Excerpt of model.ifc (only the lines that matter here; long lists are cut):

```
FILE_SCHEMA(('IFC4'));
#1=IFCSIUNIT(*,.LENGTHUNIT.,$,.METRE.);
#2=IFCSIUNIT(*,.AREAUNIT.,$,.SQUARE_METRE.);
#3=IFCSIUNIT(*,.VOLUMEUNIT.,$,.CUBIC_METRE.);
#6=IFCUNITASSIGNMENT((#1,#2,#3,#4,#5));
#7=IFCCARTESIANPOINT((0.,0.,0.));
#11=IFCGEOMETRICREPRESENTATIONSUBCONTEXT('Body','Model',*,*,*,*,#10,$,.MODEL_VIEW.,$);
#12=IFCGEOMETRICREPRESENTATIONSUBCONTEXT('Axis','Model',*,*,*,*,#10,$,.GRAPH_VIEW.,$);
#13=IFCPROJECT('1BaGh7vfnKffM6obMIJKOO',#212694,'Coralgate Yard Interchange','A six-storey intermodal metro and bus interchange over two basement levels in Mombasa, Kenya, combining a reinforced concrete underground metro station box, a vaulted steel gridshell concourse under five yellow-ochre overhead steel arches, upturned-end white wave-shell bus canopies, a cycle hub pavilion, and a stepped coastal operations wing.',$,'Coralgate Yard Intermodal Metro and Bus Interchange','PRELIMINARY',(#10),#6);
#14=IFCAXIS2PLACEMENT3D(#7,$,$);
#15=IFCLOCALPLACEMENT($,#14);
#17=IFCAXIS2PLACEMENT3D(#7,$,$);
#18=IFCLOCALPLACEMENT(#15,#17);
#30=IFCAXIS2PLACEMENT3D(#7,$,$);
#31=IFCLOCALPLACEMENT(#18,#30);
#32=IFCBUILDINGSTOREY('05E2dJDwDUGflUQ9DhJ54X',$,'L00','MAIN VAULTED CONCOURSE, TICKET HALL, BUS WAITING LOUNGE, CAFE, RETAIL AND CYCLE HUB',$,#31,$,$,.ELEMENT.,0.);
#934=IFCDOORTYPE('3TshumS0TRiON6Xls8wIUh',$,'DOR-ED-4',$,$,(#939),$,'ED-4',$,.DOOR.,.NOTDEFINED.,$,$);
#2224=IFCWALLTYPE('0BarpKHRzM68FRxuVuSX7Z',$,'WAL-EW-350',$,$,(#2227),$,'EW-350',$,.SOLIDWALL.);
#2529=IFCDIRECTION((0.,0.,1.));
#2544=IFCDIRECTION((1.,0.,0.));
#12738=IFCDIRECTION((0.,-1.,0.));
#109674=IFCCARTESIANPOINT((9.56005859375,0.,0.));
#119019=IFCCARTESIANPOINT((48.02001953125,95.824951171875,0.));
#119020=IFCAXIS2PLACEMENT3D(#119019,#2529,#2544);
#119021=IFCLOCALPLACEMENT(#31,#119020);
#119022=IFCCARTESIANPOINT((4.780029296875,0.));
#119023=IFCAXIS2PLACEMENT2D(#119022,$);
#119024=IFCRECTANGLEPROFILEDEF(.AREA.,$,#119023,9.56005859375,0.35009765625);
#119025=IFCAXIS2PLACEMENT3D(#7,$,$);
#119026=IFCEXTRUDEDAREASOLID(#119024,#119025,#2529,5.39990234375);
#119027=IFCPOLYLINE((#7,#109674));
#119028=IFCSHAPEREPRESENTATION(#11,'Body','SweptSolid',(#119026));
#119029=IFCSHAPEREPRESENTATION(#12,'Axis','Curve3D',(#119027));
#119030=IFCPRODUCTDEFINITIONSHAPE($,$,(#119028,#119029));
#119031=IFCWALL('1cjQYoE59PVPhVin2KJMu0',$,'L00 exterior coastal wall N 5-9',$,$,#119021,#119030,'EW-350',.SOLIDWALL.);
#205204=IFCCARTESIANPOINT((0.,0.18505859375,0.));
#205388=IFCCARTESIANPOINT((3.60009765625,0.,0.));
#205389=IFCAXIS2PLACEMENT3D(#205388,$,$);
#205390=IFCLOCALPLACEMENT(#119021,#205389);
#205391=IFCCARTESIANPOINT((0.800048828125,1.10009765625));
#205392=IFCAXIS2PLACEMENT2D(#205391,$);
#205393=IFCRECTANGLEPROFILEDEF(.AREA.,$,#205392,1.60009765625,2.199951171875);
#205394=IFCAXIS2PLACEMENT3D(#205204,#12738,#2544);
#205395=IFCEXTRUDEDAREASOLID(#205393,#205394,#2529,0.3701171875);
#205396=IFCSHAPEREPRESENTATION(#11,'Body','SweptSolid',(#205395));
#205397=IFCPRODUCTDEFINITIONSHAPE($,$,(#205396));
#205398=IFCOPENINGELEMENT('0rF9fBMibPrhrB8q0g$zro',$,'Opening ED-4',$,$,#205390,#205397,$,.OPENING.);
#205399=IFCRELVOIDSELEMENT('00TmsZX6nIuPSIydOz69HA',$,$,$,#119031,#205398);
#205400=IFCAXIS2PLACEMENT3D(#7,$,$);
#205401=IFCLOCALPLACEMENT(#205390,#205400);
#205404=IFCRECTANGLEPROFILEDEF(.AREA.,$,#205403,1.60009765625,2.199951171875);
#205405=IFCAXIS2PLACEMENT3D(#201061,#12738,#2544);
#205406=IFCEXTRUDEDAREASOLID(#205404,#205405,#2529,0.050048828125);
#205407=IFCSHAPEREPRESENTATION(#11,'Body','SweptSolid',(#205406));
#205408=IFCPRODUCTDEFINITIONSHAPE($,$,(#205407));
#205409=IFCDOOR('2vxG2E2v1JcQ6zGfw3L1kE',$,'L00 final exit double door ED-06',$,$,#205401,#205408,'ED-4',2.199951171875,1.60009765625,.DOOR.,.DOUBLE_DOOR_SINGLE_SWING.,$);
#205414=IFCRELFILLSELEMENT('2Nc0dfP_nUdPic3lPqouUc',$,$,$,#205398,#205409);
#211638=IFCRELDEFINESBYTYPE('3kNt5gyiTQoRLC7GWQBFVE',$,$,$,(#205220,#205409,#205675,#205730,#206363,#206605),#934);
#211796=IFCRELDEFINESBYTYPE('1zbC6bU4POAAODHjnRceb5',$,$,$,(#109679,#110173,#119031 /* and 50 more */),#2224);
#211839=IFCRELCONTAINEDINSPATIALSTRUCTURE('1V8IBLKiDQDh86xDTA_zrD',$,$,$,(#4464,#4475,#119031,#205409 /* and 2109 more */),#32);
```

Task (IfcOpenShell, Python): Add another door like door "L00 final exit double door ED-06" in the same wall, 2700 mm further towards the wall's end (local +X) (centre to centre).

```python
import ifcopenshell
import ifcopenshell.api.feature
import ifcopenshell.api.geometry
import ifcopenshell.api.root
import ifcopenshell.geom
import ifcopenshell.util.element
import ifcopenshell.util.placement
import ifcopenshell.util.shape

model = ifcopenshell.open("model.ifc")
settings = ifcopenshell.geom.settings()


def volume(element):
    """Net volume in cubic metres, openings subtracted."""
    shape = ifcopenshell.geom.create_shape(settings, element)
    return ifcopenshell.util.shape.get_volume(shape.geometry)


door = model.by_guid("2vxG2E2v1JcQ6zGfw3L1kE")
opening = door.FillsVoids[0].RelatingOpeningElement
wall = opening.VoidsElements[0].RelatingBuildingElement
before = volume(wall)
shift = ifcopenshell.util.placement.get_local_placement(wall.ObjectPlacement)[:3, 0] * 2.7

# copy_class copies the void relationship, type, container and properties, but no geometry.
new_opening = ifcopenshell.api.root.copy_class(model, product=opening)
new_opening.Representation = ifcopenshell.util.element.copy_deep(
    model, opening.Representation, exclude=["IfcGeometricRepresentationContext", "IfcRepresentationMap"]
)
new_door = ifcopenshell.api.root.copy_class(model, product=door)
new_door.Representation = ifcopenshell.util.element.copy_deep(
    model, door.Representation, exclude=["IfcGeometricRepresentationContext", "IfcRepresentationMap"]
)
new_door.Tag = None
ifcopenshell.api.feature.add_filling(model, opening=new_opening, element=new_door)

for old, new in ((opening, new_opening), (door, new_door)):
    matrix = ifcopenshell.util.placement.get_local_placement(old.ObjectPlacement)
    matrix[:3, 3] += shift
    ifcopenshell.api.geometry.edit_object_placement(model, product=new, matrix=matrix, is_si=False)

after = volume(wall)

print(f"wall volume {before:.3f} -> {after:.3f} m3")

model.write("model_v2.ifc")
```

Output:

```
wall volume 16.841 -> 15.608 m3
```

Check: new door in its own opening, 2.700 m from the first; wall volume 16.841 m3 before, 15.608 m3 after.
